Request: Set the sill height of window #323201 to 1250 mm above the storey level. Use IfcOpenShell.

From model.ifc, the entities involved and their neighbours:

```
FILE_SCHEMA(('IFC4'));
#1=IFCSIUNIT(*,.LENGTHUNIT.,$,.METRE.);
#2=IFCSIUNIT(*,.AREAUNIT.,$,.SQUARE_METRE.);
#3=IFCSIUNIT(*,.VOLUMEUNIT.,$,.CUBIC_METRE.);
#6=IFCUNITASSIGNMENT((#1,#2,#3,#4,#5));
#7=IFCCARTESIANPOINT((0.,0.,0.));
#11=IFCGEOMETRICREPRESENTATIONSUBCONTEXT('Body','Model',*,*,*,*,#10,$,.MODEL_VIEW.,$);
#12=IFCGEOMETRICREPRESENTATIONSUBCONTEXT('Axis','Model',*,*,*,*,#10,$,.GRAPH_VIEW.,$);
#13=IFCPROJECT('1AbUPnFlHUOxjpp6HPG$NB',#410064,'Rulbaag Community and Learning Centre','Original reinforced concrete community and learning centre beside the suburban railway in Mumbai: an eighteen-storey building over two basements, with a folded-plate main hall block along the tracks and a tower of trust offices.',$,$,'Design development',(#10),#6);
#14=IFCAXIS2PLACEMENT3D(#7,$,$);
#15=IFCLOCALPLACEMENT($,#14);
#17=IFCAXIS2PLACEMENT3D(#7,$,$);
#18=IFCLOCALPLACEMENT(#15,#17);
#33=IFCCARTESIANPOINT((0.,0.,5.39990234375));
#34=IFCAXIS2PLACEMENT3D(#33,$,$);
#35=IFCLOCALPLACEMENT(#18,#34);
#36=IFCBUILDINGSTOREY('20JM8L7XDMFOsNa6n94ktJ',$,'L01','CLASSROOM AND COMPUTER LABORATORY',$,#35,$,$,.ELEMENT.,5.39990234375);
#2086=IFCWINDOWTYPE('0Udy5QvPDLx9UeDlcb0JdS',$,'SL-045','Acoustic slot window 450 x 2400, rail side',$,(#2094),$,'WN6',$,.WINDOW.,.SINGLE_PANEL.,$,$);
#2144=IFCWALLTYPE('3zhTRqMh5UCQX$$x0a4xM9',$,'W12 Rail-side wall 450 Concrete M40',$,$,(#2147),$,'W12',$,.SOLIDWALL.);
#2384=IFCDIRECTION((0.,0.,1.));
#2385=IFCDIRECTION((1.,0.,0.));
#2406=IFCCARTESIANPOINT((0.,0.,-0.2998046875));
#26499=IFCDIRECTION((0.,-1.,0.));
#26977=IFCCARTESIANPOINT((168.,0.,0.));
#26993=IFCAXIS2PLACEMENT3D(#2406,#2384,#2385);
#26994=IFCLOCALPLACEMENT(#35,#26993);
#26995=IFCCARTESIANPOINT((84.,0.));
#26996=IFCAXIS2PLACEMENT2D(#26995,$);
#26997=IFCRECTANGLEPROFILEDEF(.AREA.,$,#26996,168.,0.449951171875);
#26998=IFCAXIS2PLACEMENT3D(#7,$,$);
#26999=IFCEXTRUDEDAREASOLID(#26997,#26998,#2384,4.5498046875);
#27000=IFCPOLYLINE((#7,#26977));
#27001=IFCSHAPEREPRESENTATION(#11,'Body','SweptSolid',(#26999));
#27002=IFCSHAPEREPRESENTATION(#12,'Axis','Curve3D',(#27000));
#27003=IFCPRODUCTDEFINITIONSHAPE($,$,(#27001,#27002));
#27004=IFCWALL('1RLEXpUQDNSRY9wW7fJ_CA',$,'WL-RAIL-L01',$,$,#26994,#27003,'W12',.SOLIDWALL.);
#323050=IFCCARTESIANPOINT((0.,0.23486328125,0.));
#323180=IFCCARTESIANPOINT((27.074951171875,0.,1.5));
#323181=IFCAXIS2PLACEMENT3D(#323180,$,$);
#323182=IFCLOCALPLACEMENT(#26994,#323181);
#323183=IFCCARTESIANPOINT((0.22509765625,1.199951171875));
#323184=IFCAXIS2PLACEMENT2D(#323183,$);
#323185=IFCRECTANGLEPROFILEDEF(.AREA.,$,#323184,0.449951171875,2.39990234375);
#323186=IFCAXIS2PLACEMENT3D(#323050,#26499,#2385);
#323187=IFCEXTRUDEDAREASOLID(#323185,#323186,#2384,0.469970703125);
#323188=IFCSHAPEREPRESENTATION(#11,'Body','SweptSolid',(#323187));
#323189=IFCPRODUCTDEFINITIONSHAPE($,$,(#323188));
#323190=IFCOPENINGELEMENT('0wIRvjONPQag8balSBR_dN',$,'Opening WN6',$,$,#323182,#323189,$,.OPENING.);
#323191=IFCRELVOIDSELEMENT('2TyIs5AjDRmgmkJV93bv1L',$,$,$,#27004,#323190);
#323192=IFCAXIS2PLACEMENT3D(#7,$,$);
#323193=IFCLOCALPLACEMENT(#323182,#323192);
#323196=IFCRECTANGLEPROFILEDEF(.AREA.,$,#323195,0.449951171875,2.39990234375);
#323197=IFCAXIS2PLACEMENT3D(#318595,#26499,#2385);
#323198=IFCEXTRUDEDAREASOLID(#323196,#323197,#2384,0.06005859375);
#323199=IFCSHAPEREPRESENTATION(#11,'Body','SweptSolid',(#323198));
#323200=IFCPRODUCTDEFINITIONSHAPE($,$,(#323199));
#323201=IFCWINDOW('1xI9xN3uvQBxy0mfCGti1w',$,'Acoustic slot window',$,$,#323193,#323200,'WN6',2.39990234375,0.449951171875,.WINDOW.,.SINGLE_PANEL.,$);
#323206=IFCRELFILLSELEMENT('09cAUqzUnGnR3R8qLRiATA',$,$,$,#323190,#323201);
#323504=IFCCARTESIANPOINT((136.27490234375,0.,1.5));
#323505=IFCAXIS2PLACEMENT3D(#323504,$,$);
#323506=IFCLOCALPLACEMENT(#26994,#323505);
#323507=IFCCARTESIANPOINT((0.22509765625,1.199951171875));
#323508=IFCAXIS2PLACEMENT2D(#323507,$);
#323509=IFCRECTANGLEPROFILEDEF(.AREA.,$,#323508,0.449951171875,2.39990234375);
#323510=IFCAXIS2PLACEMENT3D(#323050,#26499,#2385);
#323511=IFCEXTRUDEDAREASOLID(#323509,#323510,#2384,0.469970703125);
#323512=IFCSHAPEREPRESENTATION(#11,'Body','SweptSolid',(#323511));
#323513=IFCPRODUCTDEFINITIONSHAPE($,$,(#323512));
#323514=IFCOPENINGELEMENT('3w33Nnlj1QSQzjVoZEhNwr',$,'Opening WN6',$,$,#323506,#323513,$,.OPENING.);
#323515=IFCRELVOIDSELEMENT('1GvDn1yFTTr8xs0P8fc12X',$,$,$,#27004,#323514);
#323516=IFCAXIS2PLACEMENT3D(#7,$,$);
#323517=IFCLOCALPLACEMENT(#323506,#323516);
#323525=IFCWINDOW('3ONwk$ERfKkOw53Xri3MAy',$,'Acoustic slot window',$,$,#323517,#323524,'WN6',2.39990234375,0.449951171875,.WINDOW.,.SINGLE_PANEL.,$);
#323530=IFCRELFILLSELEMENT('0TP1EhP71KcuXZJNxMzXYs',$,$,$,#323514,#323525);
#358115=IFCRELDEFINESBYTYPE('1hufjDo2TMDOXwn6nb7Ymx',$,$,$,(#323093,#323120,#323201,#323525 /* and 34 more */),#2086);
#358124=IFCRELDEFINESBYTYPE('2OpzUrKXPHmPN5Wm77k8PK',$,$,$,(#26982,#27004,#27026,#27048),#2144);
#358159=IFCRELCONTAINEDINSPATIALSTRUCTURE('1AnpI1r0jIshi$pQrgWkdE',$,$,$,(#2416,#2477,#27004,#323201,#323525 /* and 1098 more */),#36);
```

```python
import numpy as np
import ifcopenshell
import ifcopenshell.api.geometry
import ifcopenshell.geom
import ifcopenshell.util.element
import ifcopenshell.util.placement
import ifcopenshell.util.shape
import ifcopenshell.util.unit

model = ifcopenshell.open("model.ifc")
unit_scale = ifcopenshell.util.unit.calculate_unit_scale(model)

window = model.by_id(323201)
opening = window.FillsVoids[0].RelatingOpeningElement
storey = ifcopenshell.util.element.get_container(window, ifc_class="IfcBuildingStorey")
level = ifcopenshell.util.placement.get_local_placement(storey.ObjectPlacement)[2, 3]

# The opening's origin need not be at the sill, so measure its lowest point.
shape = ifcopenshell.geom.create_shape(ifcopenshell.geom.settings(), opening)
bottom = ifcopenshell.util.shape.get_shape_bottom_elevation(shape, shape.geometry) / unit_scale
dz = level + 1.25 / unit_scale - bottom

shift = np.array([0.0, 0.0, dz])
# The window is placed relative to its opening, so it follows when the opening moves.
matrix = ifcopenshell.util.placement.get_local_placement(opening.ObjectPlacement)
matrix[:3, 3] += shift
ifcopenshell.api.geometry.edit_object_placement(
    model, product=opening, matrix=matrix, is_si=False, should_transform_children=True
)

print(f"moved by {dz * unit_scale:+.3f} m")

model.write("model_rev.ifc")
```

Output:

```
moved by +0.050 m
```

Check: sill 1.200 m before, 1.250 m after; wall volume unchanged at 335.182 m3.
